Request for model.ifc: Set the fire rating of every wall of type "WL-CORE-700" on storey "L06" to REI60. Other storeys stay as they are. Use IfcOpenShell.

First a look at what the model holds.

```python
import ifcopenshell
import ifcopenshell.util.element

model = ifcopenshell.open("model.ifc")
print(model.schema)
storey = next(s for s in model.by_type("IfcBuildingStorey") if s.Name == "L06")
walls = [e for e in ifcopenshell.util.element.get_decomposition(storey) if e.is_a("IfcWall")]
seen = {}
for e in walls:
    element_type = ifcopenshell.util.element.get_type(e)
    key = (element_type.Name if element_type != e and element_type else None, ifcopenshell.util.element.get_pset(e, "Pset_WallCommon", "FireRating"))
    seen[key] = seen.get(key, 0) + 1
for (name, value), count in sorted(seen.items(), key=str):
    print(count, "x", name, "|", value)
```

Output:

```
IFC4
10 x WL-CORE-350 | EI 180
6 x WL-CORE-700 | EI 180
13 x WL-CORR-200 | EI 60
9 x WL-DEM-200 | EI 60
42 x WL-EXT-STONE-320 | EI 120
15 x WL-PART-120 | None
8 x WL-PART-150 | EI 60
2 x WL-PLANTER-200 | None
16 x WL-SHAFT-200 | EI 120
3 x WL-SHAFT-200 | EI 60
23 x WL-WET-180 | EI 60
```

```python
import ifcopenshell
import ifcopenshell.api.pset
import ifcopenshell.util.element

model = ifcopenshell.open("model.ifc")

storey = next(s for s in model.by_type("IfcBuildingStorey") if s.Name == "L06")
walls = [e for e in ifcopenshell.util.element.get_decomposition(storey) if e.is_a("IfcWall")]

count = 0
for e in walls:
    element_type = ifcopenshell.util.element.get_type(e)
    if element_type in (None, e) or element_type.Name != "WL-CORE-700":
        continue
    # add_pset returns the element's existing set when there is one.
    pset = ifcopenshell.api.pset.add_pset(model, product=e, name="Pset_WallCommon")
    ifcopenshell.api.pset.edit_pset(model, pset=pset, properties={"FireRating": "REI60"})
    count += 1

print(count, "walls updated")

model.write("model_updated.ifc")
```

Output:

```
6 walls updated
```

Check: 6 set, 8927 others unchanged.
